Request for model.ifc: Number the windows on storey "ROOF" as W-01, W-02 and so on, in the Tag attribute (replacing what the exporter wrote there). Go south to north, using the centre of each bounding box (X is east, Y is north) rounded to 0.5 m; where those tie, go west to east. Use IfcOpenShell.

First a look at what the model holds.

```python
import ifcopenshell
import ifcopenshell.util.element
import ifcopenshell.util.placement

model = ifcopenshell.open("model.ifc")
print(model.schema)
storey = next(s for s in model.by_type("IfcBuildingStorey") if s.Name == "ROOF")
windows = [e for e in ifcopenshell.util.element.get_decomposition(storey) if e.is_a("IfcWindow")]
for e in sorted(windows, key=lambda e: e.id()):
    origin = ifcopenshell.util.placement.get_local_placement(e.ObjectPlacement)[:3, 3]
    print(e.id(), e.Tag, e.Name, origin.round(2) + 0.0, sep=" | ")
```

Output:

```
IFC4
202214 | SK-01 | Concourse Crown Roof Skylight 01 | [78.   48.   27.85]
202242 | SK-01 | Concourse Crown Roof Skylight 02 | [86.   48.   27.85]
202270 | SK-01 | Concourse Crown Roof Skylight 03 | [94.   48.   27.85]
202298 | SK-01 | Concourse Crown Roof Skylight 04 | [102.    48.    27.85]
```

```python
import ifcopenshell
import ifcopenshell.geom
import ifcopenshell.util.element
import ifcopenshell.util.shape

model = ifcopenshell.open("model.ifc")
settings = ifcopenshell.geom.settings()
settings.set("use-world-coords", True)


def centre(element):
    shape = ifcopenshell.geom.create_shape(settings, element)
    return ifcopenshell.util.shape.get_bbox_centroid(shape.geometry)


storey = next(s for s in model.by_type("IfcBuildingStorey") if s.Name == "ROOF")
windows = [e for e in ifcopenshell.util.element.get_decomposition(storey) if e.is_a("IfcWindow")]

# Insertion points can sit at a corner or the storey origin, so sort by the geometry (in metres).
centres = {e: centre(e) for e in windows}
windows.sort(key=lambda e: (round(centres[e][1] / 0.5), centres[e][0]))

for i, e in enumerate(windows, start=1):
    number = f"W-{i:02d}"
    e.Tag = number
    print(e.id(), number)

model.write("model-out.ifc")
```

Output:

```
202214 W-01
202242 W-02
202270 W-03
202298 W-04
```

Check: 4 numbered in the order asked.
